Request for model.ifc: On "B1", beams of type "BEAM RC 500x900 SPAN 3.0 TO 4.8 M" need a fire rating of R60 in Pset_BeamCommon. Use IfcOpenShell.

First a look at what the model holds.

```python
import ifcopenshell
import ifcopenshell.util.element

model = ifcopenshell.open("model.ifc")
print(model.schema)
storey = next(s for s in model.by_type("IfcBuildingStorey") if s.Name == "B1")
beams = [e for e in ifcopenshell.util.element.get_decomposition(storey) if e.is_a("IfcBeam")]
seen = {}
for e in beams:
    element_type = ifcopenshell.util.element.get_type(e)
    key = (element_type.Name if element_type != e and element_type else None, ifcopenshell.util.element.get_pset(e, "Pset_BeamCommon", "FireRating"))
    seen[key] = seen.get(key, 0) + 1
for (name, value), count in sorted(seen.items(), key=str):
    print(count, "x", name, "|", value)
```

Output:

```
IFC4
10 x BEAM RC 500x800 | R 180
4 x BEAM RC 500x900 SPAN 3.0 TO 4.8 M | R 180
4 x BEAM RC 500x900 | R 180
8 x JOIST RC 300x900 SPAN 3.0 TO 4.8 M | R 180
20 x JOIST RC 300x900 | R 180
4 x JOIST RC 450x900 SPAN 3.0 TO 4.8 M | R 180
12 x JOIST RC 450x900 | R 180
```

```python
import ifcopenshell
import ifcopenshell.api.pset
import ifcopenshell.util.element

model = ifcopenshell.open("model.ifc")

storey = next(s for s in model.by_type("IfcBuildingStorey") if s.Name == "B1")
beams = [e for e in ifcopenshell.util.element.get_decomposition(storey) if e.is_a("IfcBeam")]

count = 0
for e in beams:
    element_type = ifcopenshell.util.element.get_type(e)
    if element_type in (None, e) or element_type.Name != "BEAM RC 500x900 SPAN 3.0 TO 4.8 M":
        continue
    # add_pset returns the element's existing set when there is one.
    pset = ifcopenshell.api.pset.add_pset(model, product=e, name="Pset_BeamCommon")
    ifcopenshell.api.pset.edit_pset(model, pset=pset, properties={"FireRating": "R60"})
    count += 1

print(count, "beams updated")

model.write("model_v2.ifc")
```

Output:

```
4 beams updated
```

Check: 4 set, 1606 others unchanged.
